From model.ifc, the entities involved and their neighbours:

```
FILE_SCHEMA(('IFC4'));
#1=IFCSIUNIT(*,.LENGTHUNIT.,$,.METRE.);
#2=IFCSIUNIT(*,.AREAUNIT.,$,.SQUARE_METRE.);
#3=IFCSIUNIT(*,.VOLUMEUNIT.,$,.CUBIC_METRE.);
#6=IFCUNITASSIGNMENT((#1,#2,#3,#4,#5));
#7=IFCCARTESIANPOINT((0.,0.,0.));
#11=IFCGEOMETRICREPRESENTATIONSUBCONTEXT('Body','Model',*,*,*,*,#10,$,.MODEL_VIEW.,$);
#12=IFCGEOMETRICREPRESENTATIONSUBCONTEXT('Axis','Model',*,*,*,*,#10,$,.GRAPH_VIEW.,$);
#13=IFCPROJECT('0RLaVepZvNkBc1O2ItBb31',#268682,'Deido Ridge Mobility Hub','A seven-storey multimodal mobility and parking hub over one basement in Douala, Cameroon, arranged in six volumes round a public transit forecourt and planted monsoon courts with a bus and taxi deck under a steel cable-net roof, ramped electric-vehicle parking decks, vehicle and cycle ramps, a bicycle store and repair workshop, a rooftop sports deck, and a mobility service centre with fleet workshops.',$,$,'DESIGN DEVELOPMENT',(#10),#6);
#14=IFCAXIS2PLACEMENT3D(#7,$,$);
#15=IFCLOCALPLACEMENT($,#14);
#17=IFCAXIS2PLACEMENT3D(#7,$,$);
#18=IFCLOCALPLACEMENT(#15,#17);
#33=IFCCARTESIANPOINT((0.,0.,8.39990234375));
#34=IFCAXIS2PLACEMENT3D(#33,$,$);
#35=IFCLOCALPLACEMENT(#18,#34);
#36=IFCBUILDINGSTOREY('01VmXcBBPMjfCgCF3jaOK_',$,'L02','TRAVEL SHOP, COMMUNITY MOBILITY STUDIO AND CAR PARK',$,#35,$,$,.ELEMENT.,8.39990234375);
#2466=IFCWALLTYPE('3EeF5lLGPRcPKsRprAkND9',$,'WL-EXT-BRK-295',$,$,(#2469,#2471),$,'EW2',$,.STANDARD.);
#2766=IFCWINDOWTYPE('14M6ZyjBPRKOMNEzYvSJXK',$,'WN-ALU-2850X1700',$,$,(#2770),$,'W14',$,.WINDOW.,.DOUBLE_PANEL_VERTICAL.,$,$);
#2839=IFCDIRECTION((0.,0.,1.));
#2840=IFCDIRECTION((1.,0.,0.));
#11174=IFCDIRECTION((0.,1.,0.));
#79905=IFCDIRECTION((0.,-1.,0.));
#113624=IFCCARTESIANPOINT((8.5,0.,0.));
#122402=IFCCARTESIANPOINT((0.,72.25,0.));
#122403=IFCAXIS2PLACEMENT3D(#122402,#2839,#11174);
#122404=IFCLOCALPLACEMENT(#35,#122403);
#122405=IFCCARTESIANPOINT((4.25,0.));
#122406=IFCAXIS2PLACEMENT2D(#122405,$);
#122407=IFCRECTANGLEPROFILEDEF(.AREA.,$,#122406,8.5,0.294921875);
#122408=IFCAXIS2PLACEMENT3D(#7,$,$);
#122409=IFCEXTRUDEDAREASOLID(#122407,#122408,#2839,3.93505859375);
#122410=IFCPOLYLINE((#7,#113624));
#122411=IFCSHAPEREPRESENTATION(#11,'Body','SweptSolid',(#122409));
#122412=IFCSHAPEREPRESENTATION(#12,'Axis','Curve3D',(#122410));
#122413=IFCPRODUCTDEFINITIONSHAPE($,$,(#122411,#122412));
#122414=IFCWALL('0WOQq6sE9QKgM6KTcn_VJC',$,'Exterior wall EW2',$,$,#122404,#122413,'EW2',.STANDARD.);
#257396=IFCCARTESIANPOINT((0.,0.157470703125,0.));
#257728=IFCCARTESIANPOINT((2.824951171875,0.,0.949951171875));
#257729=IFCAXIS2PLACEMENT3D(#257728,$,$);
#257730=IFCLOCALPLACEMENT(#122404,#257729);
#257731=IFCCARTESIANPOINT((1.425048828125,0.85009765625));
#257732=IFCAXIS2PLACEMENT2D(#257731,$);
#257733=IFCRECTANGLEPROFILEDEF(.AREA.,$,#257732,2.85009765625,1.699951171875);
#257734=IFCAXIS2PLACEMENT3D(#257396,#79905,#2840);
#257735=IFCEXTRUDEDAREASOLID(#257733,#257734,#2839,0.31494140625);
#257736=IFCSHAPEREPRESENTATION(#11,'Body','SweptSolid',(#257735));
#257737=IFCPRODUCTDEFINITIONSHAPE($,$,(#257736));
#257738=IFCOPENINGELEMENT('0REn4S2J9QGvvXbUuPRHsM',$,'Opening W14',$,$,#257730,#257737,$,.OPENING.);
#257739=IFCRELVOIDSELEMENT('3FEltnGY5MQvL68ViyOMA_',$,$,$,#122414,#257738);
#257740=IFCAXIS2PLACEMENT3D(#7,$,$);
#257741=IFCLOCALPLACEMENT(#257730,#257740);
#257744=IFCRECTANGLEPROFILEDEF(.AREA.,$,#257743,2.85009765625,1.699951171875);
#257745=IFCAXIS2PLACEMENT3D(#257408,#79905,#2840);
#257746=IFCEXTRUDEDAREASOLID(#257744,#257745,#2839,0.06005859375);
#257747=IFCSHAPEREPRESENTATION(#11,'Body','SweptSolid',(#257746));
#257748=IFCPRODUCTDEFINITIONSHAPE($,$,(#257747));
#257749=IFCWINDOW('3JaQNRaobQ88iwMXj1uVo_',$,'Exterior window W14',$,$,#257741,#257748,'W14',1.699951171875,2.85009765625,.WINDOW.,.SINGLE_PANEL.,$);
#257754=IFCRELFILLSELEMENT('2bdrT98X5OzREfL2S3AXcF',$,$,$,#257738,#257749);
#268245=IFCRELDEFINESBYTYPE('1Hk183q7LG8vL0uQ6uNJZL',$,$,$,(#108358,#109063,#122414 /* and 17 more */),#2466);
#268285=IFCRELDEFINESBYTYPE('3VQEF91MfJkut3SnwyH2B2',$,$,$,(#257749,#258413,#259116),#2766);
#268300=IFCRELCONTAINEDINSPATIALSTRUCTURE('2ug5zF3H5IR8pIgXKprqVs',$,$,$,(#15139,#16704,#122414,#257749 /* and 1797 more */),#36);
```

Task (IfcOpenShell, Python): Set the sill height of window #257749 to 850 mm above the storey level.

```python
import numpy as np
import ifcopenshell
import ifcopenshell.api.geometry
import ifcopenshell.geom
import ifcopenshell.util.element
import ifcopenshell.util.placement
import ifcopenshell.util.shape
import ifcopenshell.util.unit

model = ifcopenshell.open("model.ifc")
unit_scale = ifcopenshell.util.unit.calculate_unit_scale(model)

window = model.by_guid("3JaQNRaobQ88iwMXj1uVo_")
opening = window.FillsVoids[0].RelatingOpeningElement
storey = ifcopenshell.util.element.get_container(window, ifc_class="IfcBuildingStorey")
level = ifcopenshell.util.placement.get_local_placement(storey.ObjectPlacement)[2, 3]

# The opening's origin need not be at the sill, so measure its lowest point.
shape = ifcopenshell.geom.create_shape(ifcopenshell.geom.settings(), opening)
bottom = ifcopenshell.util.shape.get_shape_bottom_elevation(shape, shape.geometry) / unit_scale
dz = level + 0.85 - bottom

shift = np.array([0.0, 0.0, dz])
# The window is placed relative to its opening, so it follows when the opening moves.
matrix = ifcopenshell.util.placement.get_local_placement(opening.ObjectPlacement)
matrix[:3, 3] += shift
ifcopenshell.api.geometry.edit_object_placement(
    model, product=opening, matrix=matrix, is_si=False, should_transform_children=True
)

print(f"moved by {dz * unit_scale:+.3f} m")

model.write("model-out.ifc")
```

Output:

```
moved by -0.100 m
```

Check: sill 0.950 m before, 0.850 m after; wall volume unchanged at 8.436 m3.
